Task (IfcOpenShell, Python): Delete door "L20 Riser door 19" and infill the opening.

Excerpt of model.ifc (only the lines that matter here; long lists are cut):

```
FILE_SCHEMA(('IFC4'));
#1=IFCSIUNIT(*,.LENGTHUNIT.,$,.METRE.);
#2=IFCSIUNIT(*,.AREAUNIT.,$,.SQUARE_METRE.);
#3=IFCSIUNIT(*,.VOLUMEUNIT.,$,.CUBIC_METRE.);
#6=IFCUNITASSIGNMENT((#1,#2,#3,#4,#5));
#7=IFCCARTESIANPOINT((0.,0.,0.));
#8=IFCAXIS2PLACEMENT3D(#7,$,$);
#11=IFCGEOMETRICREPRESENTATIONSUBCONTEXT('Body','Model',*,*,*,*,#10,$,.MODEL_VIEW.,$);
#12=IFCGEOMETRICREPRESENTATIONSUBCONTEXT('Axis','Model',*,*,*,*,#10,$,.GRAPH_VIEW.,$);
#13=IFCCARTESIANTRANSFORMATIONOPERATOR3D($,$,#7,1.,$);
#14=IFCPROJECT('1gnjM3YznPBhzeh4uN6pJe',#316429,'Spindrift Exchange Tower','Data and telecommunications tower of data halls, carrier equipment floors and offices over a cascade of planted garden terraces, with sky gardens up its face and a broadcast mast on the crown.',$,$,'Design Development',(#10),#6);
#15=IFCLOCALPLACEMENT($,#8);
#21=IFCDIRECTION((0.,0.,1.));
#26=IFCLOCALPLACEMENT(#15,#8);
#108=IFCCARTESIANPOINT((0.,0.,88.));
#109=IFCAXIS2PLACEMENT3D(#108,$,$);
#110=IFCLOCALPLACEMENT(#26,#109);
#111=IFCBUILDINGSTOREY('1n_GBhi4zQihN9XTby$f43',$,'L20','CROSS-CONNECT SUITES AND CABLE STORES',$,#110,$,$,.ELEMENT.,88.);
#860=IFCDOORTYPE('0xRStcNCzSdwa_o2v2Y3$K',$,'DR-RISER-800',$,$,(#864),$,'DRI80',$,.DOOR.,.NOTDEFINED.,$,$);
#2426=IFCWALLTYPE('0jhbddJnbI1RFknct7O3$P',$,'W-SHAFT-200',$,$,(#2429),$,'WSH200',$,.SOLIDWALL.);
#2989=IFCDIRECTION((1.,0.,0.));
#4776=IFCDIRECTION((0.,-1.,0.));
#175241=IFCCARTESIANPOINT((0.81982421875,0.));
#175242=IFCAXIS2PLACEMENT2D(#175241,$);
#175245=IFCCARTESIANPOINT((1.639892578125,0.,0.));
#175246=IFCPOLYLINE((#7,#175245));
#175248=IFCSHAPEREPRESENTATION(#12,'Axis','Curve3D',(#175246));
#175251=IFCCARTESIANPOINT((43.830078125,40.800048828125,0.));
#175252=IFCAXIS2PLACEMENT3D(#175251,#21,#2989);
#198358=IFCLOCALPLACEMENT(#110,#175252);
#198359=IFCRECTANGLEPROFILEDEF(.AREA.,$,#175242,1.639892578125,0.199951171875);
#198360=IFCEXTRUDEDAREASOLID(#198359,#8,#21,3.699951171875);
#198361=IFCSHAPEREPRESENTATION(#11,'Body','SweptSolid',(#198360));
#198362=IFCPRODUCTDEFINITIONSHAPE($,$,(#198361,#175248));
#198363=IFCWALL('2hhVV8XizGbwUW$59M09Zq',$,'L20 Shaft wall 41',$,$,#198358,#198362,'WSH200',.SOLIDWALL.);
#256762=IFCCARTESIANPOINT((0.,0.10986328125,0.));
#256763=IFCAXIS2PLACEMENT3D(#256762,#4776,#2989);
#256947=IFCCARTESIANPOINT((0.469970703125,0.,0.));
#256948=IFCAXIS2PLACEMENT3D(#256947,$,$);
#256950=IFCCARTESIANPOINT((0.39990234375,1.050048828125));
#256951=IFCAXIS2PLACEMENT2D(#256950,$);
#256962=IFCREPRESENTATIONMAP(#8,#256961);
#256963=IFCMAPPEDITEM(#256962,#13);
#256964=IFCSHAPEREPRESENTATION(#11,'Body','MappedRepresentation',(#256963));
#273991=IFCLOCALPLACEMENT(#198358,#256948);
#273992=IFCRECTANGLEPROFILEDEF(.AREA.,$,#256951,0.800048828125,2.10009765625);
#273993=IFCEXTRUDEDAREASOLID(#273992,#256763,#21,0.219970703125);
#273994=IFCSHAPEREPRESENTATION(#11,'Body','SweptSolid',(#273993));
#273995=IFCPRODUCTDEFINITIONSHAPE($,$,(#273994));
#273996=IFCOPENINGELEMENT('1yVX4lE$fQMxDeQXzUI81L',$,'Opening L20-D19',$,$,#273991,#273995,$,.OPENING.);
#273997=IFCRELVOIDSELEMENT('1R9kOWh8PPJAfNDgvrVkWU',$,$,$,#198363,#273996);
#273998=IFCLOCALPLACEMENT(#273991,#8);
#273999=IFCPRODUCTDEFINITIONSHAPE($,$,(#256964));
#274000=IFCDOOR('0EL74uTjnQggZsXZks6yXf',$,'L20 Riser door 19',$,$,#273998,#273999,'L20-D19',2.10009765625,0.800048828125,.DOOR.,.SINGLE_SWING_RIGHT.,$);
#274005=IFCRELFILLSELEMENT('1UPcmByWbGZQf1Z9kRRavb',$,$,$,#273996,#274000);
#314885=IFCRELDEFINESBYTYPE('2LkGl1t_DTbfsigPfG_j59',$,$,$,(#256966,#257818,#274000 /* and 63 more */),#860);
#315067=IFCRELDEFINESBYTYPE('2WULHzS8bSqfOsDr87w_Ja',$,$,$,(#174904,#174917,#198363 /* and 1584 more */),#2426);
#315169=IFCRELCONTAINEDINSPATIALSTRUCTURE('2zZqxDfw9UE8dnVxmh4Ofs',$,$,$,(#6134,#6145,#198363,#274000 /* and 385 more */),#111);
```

```python
import ifcopenshell
import ifcopenshell.api.feature
import ifcopenshell.api.root
import ifcopenshell.geom
import ifcopenshell.util.shape

model = ifcopenshell.open("model.ifc")
settings = ifcopenshell.geom.settings()


def volume(element):
    """Net volume in cubic metres, openings subtracted."""
    shape = ifcopenshell.geom.create_shape(settings, element)
    return ifcopenshell.util.shape.get_volume(shape.geometry)


door = model.by_guid("0EL74uTjnQggZsXZks6yXf")
opening = door.FillsVoids[0].RelatingOpeningElement
wall = opening.VoidsElements[0].RelatingBuildingElement
before = volume(wall)

ifcopenshell.api.root.remove_product(model, product=door)
ifcopenshell.api.feature.remove_feature(model, feature=opening)

after = volume(wall)

print(f"wall volume {before:.3f} -> {after:.3f} m3")

model.write("model_edited.ifc")
```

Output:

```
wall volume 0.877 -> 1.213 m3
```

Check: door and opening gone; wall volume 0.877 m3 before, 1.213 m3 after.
